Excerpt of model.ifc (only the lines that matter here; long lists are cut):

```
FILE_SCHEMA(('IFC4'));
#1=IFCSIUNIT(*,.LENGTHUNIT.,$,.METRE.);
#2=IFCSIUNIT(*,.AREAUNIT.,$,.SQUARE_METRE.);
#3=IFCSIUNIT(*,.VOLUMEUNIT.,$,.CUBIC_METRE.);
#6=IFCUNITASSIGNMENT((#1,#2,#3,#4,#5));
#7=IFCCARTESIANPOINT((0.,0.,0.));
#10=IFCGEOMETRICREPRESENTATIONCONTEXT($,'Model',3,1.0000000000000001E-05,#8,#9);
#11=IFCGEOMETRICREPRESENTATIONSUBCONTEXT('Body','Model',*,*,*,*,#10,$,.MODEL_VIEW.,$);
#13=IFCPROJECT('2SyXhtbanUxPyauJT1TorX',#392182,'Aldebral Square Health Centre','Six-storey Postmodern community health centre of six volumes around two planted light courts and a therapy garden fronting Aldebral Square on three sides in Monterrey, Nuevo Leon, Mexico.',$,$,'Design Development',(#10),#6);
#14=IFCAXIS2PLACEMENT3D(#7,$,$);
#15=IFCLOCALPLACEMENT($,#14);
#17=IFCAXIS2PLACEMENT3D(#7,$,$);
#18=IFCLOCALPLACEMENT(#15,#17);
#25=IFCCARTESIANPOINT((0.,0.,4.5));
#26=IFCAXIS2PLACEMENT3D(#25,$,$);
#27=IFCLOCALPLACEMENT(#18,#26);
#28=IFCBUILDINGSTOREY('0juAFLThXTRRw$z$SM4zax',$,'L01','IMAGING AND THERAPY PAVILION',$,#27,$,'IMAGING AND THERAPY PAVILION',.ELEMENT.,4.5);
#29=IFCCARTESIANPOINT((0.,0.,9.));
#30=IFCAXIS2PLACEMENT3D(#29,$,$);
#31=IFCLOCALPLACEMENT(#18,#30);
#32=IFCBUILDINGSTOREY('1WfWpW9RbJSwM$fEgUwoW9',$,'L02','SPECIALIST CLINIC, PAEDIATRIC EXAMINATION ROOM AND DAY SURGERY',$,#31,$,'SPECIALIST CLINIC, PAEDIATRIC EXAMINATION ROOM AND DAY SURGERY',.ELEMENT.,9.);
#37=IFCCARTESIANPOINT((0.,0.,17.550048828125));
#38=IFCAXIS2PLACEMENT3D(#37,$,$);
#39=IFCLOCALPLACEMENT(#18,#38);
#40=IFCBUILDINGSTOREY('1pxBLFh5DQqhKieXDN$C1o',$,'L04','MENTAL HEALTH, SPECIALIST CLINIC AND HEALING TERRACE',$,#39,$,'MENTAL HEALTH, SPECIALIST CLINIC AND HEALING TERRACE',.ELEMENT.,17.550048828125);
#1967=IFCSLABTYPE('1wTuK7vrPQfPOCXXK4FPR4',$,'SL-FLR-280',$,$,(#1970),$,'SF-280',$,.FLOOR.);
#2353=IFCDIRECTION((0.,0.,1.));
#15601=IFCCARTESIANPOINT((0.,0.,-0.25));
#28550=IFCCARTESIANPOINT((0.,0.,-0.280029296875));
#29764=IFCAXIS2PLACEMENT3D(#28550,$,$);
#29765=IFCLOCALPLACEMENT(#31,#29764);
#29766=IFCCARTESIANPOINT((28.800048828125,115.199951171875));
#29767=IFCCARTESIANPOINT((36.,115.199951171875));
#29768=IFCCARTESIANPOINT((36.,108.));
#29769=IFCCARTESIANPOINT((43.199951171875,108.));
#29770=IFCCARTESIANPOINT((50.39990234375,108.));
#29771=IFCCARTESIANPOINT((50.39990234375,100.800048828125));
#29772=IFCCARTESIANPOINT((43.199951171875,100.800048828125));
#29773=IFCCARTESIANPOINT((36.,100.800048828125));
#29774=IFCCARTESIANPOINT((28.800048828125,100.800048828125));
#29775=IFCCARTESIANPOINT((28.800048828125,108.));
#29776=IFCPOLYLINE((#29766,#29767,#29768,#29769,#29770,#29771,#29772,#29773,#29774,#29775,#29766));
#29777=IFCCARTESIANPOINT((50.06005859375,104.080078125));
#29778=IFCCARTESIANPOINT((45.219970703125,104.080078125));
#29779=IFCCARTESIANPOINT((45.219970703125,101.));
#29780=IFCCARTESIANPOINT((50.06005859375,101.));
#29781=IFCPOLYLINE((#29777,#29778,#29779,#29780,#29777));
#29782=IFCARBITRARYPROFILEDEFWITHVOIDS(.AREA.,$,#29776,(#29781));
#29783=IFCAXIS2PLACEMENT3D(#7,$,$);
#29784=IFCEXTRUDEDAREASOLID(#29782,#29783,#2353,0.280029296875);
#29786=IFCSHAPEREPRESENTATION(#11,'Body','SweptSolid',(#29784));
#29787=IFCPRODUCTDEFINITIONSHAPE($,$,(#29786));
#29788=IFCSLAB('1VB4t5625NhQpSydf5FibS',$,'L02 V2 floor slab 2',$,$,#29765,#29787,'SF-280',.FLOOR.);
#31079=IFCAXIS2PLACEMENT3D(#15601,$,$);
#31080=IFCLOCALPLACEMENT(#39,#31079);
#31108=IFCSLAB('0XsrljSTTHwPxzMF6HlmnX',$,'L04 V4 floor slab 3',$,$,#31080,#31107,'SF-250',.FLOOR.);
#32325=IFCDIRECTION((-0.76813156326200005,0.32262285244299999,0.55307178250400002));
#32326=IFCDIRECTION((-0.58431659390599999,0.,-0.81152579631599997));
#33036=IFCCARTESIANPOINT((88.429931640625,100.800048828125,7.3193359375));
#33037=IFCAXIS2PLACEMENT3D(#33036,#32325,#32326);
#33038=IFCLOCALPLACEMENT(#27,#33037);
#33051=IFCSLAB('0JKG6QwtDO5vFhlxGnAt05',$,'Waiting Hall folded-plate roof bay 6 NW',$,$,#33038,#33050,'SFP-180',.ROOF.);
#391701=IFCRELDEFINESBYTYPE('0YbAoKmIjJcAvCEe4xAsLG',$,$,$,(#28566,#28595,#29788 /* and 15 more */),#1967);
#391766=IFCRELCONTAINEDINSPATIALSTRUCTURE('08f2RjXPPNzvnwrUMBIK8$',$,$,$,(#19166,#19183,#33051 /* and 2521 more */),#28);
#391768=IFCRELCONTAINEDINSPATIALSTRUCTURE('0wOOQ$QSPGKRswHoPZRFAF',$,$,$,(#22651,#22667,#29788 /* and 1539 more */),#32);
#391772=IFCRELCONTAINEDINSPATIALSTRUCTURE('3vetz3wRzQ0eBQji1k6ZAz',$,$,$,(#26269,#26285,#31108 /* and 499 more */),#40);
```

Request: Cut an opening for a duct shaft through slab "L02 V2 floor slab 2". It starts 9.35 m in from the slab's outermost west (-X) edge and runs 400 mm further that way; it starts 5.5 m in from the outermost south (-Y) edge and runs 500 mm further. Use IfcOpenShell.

```python
import numpy as np
import ifcopenshell
import ifcopenshell.api.feature
import ifcopenshell.api.geometry
import ifcopenshell.api.root
import ifcopenshell.geom
import ifcopenshell.util.placement
import ifcopenshell.util.representation
import ifcopenshell.util.shape
import ifcopenshell.util.unit

model = ifcopenshell.open("model.ifc")
unit_scale = ifcopenshell.util.unit.calculate_unit_scale(model)
settings = ifcopenshell.geom.settings()


def volume(element):
    """Net volume in cubic metres, openings subtracted."""
    shape = ifcopenshell.geom.create_shape(settings, element)
    return ifcopenshell.util.shape.get_volume(shape.geometry)


slab = model.by_guid("1VB4t5625NhQpSydf5FibS")
before = volume(slab)

# Extent in the slab's own axes, in metres. The edges named are its -X and -Y sides.
slab_shape = ifcopenshell.geom.create_shape(settings, slab)
vertices = ifcopenshell.util.shape.get_vertices(slab_shape.geometry)
x_min, y_min, bottom = vertices.min(axis=0)
top = vertices[:, 2].max()

opening = ifcopenshell.api.root.create_entity(model, ifc_class="IfcOpeningElement", name="Duct shaft opening", predefined_type="OPENING")
context = ifcopenshell.util.representation.get_context(model, "Model", "Body", "MODEL_VIEW")
width, depth = 0.4, 0.5
outline = [(0.0, 0.0), (width, 0.0), (width, depth), (0.0, depth), (0.0, 0.0)]
# Overshoot both faces by 50 mm so the cut is clean.
shape = ifcopenshell.api.geometry.add_slab_representation(
    model, context=context, depth=top - bottom + 0.1, polyline=outline
)
ifcopenshell.api.geometry.assign_representation(model, product=opening, representation=shape)

matrix = ifcopenshell.util.placement.get_local_placement(slab.ObjectPlacement)
matrix[:, 3] = matrix @ np.append(np.array([x_min + 9.35, y_min + 5.5, bottom - 0.05]) / unit_scale, 1.0)
ifcopenshell.api.geometry.edit_object_placement(model, product=opening, matrix=matrix, is_si=False)
ifcopenshell.api.feature.add_feature(model, feature=opening, element=slab)

after = volume(slab)

print(f"slab volume {before:.3f} -> {after:.3f} m3")

model.write("model_updated.ifc")
```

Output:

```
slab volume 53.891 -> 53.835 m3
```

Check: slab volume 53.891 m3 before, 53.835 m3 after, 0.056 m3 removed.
